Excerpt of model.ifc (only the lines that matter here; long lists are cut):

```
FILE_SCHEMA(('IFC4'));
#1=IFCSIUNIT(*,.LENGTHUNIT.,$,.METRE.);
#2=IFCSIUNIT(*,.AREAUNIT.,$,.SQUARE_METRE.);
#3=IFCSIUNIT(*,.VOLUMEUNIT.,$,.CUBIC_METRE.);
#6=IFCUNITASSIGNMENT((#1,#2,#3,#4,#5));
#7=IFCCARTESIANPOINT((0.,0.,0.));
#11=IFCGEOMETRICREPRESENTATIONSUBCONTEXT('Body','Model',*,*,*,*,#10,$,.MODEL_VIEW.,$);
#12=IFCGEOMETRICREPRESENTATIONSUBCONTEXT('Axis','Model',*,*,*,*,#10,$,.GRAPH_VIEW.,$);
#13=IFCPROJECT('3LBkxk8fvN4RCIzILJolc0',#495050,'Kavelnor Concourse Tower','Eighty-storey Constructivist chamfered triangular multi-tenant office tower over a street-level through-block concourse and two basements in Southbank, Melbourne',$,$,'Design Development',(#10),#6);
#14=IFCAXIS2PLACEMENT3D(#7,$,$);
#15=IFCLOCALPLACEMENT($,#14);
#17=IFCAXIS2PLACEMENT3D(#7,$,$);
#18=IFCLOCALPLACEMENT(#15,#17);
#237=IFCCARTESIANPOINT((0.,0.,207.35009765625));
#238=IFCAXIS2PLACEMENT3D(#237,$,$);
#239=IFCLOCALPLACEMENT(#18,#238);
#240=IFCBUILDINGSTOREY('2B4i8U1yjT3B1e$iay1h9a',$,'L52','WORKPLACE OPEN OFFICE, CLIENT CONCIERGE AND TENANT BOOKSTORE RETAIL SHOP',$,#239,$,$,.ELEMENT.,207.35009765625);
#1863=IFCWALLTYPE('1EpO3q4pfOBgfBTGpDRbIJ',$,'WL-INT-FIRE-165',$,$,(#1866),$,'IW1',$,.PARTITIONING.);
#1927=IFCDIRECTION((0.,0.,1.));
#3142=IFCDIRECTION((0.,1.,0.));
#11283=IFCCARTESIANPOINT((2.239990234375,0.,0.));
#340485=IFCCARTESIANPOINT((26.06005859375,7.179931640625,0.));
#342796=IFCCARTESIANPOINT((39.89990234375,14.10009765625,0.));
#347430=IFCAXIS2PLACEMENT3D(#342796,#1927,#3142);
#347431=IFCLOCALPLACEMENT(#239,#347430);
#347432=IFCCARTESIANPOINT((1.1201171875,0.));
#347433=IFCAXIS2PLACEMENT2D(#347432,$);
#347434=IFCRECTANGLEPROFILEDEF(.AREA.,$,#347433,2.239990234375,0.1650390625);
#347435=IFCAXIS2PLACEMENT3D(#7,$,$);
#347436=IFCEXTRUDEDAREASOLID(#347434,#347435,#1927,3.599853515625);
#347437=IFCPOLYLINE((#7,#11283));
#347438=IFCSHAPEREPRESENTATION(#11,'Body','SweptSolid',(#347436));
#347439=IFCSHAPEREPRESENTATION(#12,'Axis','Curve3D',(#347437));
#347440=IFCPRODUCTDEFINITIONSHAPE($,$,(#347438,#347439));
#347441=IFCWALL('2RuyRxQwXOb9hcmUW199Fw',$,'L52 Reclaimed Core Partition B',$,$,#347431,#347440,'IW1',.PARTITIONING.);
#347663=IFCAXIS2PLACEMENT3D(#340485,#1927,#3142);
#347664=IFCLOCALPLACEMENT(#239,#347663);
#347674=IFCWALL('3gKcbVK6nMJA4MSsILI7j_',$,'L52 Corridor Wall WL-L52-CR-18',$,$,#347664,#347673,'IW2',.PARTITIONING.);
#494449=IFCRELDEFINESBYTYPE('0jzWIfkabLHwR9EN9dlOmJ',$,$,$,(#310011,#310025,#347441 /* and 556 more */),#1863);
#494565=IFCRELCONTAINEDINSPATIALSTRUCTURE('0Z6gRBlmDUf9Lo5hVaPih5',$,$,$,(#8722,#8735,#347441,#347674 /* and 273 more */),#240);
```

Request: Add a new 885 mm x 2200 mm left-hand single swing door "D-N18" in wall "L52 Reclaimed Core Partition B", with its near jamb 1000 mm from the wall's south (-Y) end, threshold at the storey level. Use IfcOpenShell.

```python
import numpy as np
import ifcopenshell
import ifcopenshell.api.feature
import ifcopenshell.api.geometry
import ifcopenshell.api.root
import ifcopenshell.api.spatial
import ifcopenshell.geom
import ifcopenshell.util.element
import ifcopenshell.util.placement
import ifcopenshell.util.representation
import ifcopenshell.util.shape
import ifcopenshell.util.unit

model = ifcopenshell.open("model.ifc")
unit_scale = ifcopenshell.util.unit.calculate_unit_scale(model)
settings = ifcopenshell.geom.settings()


def volume(element):
    """Net volume in cubic metres, openings subtracted."""
    shape = ifcopenshell.geom.create_shape(settings, element)
    return ifcopenshell.util.shape.get_volume(shape.geometry)


wall = model.by_guid("2RuyRxQwXOb9hcmUW199Fw")
storey = ifcopenshell.util.element.get_container(wall, ifc_class="IfcBuildingStorey")
context = ifcopenshell.util.representation.get_context(model, "Model", "Body", "MODEL_VIEW")
before = volume(wall)

width, height, from_end, sill = 0.885, 2.2, 1, 0.0  # metres

# The wall runs along its own X axis, and the end named is its -X end.
wall_shape = ifcopenshell.geom.create_shape(settings, wall)
x, y, z = ifcopenshell.util.shape.get_vertices(wall_shape.geometry).T
start = x.min() + from_end
face, thickness = float(y.min()), float(y.max() - y.min())
wall_matrix = ifcopenshell.util.placement.get_local_placement(wall.ObjectPlacement)
level = ifcopenshell.util.placement.get_local_placement(storey.ObjectPlacement)[2, 3]


def in_wall(x, y):
    """Placement at x, y metres in the wall's axes, at sill height."""
    matrix = wall_matrix.copy()
    matrix[:, 3] = wall_matrix @ np.array([x / unit_scale, y / unit_scale, 0.0, 1.0])
    matrix[2, 3] = level + sill / unit_scale
    return matrix


# Opening: a box that overshoots both wall faces by 50 mm.
opening = ifcopenshell.api.root.create_entity(model, ifc_class="IfcOpeningElement", predefined_type="OPENING")
box = ifcopenshell.api.geometry.add_wall_representation(
    model, context=context, length=width, height=height, thickness=thickness + 0.1
)
ifcopenshell.api.geometry.assign_representation(model, product=opening, representation=box)
ifcopenshell.api.geometry.edit_object_placement(model, product=opening, matrix=in_wall(start, face - 0.05), is_si=False)
ifcopenshell.api.feature.add_feature(model, feature=opening, element=wall)

door = ifcopenshell.api.root.create_entity(model, ifc_class="IfcDoor", name="D-N18", predefined_type="DOOR")
door.OverallWidth, door.OverallHeight = width / unit_scale, height / unit_scale
door.OperationType = "SINGLE_SWING_LEFT"
body = ifcopenshell.api.geometry.add_door_representation(
    model,
    context=context,
    overall_width=door.OverallWidth,
    overall_height=door.OverallHeight,
    operation_type="SINGLE_SWING_LEFT",
    lining_properties={"LiningDepth": thickness / unit_scale, "ThresholdDepth": thickness / unit_scale},
)
ifcopenshell.api.geometry.assign_representation(model, product=door, representation=body)
ifcopenshell.api.spatial.assign_container(model, products=[door], relating_structure=storey)
ifcopenshell.api.feature.add_filling(model, opening=opening, element=door)

# The lining spans the wall, so the door starts at the wall face.
ifcopenshell.api.geometry.edit_object_placement(model, product=door, matrix=in_wall(start, face), is_si=False)

after = volume(wall)

print(f"wall volume {before:.3f} -> {after:.3f} m3")

model.write("model_rev.ifc")
```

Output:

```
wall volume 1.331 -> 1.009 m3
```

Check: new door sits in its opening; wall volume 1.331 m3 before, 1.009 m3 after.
